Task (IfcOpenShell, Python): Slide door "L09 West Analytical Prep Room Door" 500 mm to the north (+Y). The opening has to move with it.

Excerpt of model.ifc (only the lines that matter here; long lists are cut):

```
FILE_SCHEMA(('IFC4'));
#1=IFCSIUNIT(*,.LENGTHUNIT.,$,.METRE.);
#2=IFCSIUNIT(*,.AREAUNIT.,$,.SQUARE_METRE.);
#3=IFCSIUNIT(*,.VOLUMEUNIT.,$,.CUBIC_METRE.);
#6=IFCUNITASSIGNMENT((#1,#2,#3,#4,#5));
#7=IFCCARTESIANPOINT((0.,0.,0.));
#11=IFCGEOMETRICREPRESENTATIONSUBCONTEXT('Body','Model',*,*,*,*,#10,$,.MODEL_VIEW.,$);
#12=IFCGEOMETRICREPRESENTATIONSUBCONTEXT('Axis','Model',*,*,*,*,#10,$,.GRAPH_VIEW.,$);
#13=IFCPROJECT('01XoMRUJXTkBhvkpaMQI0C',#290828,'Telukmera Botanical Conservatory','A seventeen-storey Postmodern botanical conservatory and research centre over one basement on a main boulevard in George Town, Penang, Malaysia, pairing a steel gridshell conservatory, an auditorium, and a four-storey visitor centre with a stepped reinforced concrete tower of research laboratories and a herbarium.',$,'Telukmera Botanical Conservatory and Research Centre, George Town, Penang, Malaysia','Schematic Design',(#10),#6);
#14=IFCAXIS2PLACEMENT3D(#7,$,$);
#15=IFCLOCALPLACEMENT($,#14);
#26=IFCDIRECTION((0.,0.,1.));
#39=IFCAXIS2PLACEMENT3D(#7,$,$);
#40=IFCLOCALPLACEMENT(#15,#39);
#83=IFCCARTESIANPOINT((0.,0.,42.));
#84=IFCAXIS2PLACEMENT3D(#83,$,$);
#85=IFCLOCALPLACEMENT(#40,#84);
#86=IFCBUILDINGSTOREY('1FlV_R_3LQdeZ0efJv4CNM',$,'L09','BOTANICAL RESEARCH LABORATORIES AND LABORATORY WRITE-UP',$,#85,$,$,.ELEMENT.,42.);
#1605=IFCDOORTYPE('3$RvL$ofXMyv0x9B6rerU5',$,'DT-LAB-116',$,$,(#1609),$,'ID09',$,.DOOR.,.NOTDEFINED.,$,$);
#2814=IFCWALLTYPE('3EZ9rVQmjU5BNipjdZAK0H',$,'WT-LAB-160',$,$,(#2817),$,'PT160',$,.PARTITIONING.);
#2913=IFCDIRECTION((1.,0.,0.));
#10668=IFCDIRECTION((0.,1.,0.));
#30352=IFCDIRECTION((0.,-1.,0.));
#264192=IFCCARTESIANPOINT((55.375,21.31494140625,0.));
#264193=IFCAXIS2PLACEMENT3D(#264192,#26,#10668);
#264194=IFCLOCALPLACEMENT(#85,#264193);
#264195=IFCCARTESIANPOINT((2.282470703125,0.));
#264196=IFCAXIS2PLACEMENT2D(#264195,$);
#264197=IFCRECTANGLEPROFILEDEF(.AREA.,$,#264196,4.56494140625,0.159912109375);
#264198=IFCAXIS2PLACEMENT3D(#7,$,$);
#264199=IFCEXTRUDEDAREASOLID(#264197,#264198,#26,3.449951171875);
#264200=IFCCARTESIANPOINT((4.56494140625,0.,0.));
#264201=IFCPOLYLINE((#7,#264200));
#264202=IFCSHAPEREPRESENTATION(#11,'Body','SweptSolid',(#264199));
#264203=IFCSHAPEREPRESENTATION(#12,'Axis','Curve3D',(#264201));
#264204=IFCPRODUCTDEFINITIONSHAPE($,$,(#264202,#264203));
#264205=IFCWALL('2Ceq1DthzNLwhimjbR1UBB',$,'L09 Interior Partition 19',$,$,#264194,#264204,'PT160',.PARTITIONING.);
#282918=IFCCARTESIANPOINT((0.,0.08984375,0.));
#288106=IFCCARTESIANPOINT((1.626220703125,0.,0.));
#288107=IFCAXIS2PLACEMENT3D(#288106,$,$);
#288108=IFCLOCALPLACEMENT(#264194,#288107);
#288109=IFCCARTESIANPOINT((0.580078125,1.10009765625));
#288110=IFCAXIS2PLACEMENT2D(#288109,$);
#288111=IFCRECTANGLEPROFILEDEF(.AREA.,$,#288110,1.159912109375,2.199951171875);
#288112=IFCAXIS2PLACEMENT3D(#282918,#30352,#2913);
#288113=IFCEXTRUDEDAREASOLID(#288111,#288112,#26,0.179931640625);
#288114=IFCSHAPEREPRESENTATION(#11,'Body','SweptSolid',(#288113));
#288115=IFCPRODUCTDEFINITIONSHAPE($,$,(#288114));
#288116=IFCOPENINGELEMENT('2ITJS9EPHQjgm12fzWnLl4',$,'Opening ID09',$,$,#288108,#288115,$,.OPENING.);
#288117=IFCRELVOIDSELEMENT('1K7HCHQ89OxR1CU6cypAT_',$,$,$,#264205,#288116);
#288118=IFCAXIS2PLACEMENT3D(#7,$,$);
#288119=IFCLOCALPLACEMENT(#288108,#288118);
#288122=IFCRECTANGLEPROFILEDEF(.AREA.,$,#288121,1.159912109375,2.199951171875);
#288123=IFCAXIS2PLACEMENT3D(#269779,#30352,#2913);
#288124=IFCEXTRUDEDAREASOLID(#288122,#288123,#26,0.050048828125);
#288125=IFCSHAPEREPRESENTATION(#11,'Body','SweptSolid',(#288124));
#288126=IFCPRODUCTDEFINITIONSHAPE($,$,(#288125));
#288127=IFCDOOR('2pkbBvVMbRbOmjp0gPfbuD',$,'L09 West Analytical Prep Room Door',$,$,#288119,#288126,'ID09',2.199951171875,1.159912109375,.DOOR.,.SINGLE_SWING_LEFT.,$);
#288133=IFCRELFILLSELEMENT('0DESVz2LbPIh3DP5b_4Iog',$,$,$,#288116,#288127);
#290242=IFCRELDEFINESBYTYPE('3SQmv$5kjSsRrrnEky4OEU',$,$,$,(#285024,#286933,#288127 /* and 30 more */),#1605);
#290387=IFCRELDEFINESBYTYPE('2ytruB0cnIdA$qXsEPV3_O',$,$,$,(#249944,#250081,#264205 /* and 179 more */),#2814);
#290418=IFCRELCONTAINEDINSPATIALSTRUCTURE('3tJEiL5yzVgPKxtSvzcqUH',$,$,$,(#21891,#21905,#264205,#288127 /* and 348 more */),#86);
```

```python
import ifcopenshell
import ifcopenshell.api.geometry
import ifcopenshell.util.placement

model = ifcopenshell.open("model.ifc")

door = model.by_guid("2pkbBvVMbRbOmjp0gPfbuD")
opening = door.FillsVoids[0].RelatingOpeningElement
wall = opening.VoidsElements[0].RelatingBuildingElement

wall_matrix = ifcopenshell.util.placement.get_local_placement(wall.ObjectPlacement)
shift = wall_matrix[:3, 0] * 0.5
before = ifcopenshell.util.placement.get_local_placement(door.ObjectPlacement)[:3, 3].copy()

# The door is placed relative to its opening, so it follows when the opening moves.
matrix = ifcopenshell.util.placement.get_local_placement(opening.ObjectPlacement)
matrix[:3, 3] += shift
ifcopenshell.api.geometry.edit_object_placement(
    model, product=opening, matrix=matrix, is_si=False, should_transform_children=True
)

after = ifcopenshell.util.placement.get_local_placement(door.ObjectPlacement)[:3, 3]
print("door moved by", (after - before).round(3) + 0.0)

model.write("model-out.ifc")
```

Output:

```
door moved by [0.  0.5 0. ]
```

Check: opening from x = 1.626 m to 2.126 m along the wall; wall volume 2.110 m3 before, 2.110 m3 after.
